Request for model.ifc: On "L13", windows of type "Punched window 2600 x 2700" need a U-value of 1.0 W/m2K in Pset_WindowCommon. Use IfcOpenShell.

First a look at what the model holds.

```python
import ifcopenshell
import ifcopenshell.util.element

model = ifcopenshell.open("model.ifc")
print(model.schema)
storey = next(s for s in model.by_type("IfcBuildingStorey") if s.Name == "L13")
windows = [e for e in ifcopenshell.util.element.get_decomposition(storey) if e.is_a("IfcWindow")]
seen = {}
for e in windows:
    element_type = ifcopenshell.util.element.get_type(e)
    key = (element_type.Name if element_type != e and element_type else None, ifcopenshell.util.element.get_pset(e, "Pset_WindowCommon", "ThermalTransmittance"))
    seen[key] = seen.get(key, 0) + 1
for (name, value), count in sorted(seen.items(), key=str):
    print(count, "x", name, "|", value)
```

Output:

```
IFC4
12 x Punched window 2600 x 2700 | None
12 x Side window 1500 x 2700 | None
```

```python
import ifcopenshell
import ifcopenshell.api.pset
import ifcopenshell.util.element

model = ifcopenshell.open("model.ifc")

storey = next(s for s in model.by_type("IfcBuildingStorey") if s.Name == "L13")
windows = [e for e in ifcopenshell.util.element.get_decomposition(storey) if e.is_a("IfcWindow")]

count = 0
for e in windows:
    element_type = ifcopenshell.util.element.get_type(e)
    if element_type in (None, e) or element_type.Name != "Punched window 2600 x 2700":
        continue
    # add_pset returns the element's existing set when there is one.
    pset = ifcopenshell.api.pset.add_pset(model, product=e, name="Pset_WindowCommon")
    ifcopenshell.api.pset.edit_pset(model, pset=pset, properties={"ThermalTransmittance": 1.0})
    count += 1

print(count, "windows updated")

model.write("model_v2.ifc")
```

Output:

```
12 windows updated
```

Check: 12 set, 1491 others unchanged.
